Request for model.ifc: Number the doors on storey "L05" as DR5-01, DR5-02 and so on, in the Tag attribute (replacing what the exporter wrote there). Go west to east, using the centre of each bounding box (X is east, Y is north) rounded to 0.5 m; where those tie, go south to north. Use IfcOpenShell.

First a look at what the model holds.

```python
import ifcopenshell
import ifcopenshell.util.element
import ifcopenshell.util.placement

model = ifcopenshell.open("model.ifc")
print(model.schema)
storey = next(s for s in model.by_type("IfcBuildingStorey") if s.Name == "L05")
doors = [e for e in ifcopenshell.util.element.get_decomposition(storey) if e.is_a("IfcDoor")]
for e in sorted(doors, key=lambda e: e.id()):
    origin = ifcopenshell.util.placement.get_local_placement(e.ObjectPlacement)[:3, 3]
    print(e.id(), e.Tag, e.Name, origin.round(2) + 0.0, sep=" | ")
```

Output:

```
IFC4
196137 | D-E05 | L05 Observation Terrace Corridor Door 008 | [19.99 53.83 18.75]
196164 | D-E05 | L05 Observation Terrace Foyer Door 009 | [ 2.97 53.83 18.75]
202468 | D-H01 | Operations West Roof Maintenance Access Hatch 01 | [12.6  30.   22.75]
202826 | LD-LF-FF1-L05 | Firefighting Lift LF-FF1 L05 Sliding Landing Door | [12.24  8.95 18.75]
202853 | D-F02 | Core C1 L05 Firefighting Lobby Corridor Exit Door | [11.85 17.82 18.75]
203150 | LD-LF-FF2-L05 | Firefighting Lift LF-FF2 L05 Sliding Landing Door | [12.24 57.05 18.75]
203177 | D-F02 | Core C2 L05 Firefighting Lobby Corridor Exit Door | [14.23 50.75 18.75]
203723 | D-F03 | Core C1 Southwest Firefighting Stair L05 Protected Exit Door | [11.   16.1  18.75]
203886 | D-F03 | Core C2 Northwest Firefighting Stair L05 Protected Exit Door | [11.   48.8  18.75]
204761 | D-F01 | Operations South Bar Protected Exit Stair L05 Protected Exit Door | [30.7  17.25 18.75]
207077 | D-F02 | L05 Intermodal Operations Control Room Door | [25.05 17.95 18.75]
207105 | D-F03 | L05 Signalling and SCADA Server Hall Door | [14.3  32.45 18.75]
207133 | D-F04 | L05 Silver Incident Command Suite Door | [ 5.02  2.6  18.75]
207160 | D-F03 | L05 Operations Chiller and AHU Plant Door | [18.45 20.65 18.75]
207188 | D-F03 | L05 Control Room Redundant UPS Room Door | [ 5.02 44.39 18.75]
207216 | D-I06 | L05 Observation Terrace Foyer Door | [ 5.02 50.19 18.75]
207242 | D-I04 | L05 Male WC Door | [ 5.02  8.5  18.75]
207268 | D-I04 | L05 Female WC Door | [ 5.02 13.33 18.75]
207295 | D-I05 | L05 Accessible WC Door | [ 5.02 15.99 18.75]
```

```python
import ifcopenshell
import ifcopenshell.geom
import ifcopenshell.util.element
import ifcopenshell.util.shape

model = ifcopenshell.open("model.ifc")
settings = ifcopenshell.geom.settings()
settings.set("use-world-coords", True)


def centre(element):
    shape = ifcopenshell.geom.create_shape(settings, element)
    return ifcopenshell.util.shape.get_bbox_centroid(shape.geometry)


storey = next(s for s in model.by_type("IfcBuildingStorey") if s.Name == "L05")
doors = [e for e in ifcopenshell.util.element.get_decomposition(storey) if e.is_a("IfcDoor")]

# Insertion points can sit at a corner or the storey origin, so sort by the geometry (in metres).
centres = {e: centre(e) for e in doors}
doors.sort(key=lambda e: (round(centres[e][0] / 0.5), centres[e][1]))

for i, e in enumerate(doors, start=1):
    number = f"DR5-{i:02d}"
    e.Tag = number
    print(e.id(), number)

model.write("model_v2.ifc")
```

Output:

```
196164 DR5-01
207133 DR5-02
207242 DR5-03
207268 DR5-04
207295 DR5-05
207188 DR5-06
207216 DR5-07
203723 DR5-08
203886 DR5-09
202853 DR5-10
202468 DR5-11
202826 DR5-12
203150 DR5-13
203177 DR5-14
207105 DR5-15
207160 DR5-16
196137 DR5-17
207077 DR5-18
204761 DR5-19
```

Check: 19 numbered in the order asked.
